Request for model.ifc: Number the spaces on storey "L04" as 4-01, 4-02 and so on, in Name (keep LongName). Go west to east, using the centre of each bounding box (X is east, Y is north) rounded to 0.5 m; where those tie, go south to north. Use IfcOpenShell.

First a look at what the model holds.

```python
import ifcopenshell
import ifcopenshell.util.element
import ifcopenshell.util.placement

model = ifcopenshell.open("model.ifc")
print(model.schema)
storey = next(s for s in model.by_type("IfcBuildingStorey") if s.Name == "L04")
spaces = [e for e in ifcopenshell.util.element.get_decomposition(storey) if e.is_a("IfcSpace")]
for e in sorted(spaces, key=lambda e: e.id()):
    origin = ifcopenshell.util.placement.get_local_placement(e.ObjectPlacement)[:3, 3]
    print(e.id(), e.Name, e.LongName, origin.round(2) + 0.0, sep=" | ")
```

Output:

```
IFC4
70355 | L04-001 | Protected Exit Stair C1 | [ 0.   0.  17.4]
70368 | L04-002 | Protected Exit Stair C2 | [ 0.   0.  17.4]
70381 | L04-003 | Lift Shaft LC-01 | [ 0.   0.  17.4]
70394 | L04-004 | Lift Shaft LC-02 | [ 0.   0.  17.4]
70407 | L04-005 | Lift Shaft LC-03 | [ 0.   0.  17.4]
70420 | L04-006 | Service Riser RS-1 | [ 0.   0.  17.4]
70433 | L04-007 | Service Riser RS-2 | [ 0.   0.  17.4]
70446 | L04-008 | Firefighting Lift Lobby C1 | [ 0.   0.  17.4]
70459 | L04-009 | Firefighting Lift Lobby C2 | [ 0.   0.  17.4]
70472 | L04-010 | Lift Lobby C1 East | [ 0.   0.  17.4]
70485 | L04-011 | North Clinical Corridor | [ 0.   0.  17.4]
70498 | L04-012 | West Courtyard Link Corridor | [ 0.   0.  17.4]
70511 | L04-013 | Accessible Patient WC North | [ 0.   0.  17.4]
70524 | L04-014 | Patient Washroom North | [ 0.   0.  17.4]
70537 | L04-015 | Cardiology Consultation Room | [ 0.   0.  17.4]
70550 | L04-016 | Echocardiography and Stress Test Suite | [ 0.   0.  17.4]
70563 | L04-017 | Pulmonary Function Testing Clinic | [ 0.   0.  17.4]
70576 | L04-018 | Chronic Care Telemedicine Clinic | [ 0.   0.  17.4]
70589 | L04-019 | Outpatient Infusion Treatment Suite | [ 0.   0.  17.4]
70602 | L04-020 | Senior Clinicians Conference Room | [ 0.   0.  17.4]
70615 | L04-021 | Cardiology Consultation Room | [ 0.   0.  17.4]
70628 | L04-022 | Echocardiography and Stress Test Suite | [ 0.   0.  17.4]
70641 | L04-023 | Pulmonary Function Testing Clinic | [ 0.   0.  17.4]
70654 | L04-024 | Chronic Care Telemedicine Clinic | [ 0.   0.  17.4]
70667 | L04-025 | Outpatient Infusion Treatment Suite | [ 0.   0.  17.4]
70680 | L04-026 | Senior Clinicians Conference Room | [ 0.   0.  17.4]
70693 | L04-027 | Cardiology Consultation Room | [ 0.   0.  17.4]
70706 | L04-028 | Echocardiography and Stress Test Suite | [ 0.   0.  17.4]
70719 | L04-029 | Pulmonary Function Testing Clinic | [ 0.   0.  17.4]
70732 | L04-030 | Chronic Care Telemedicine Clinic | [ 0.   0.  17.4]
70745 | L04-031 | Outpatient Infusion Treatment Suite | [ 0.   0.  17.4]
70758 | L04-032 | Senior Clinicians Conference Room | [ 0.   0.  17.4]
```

```python
import ifcopenshell
import ifcopenshell.geom
import ifcopenshell.util.element
import ifcopenshell.util.shape

model = ifcopenshell.open("model.ifc")
settings = ifcopenshell.geom.settings()
settings.set("use-world-coords", True)


def centre(element):
    shape = ifcopenshell.geom.create_shape(settings, element)
    return ifcopenshell.util.shape.get_bbox_centroid(shape.geometry)


storey = next(s for s in model.by_type("IfcBuildingStorey") if s.Name == "L04")
spaces = [e for e in ifcopenshell.util.element.get_decomposition(storey) if e.is_a("IfcSpace")]

# Insertion points can sit at a corner or the storey origin, so sort by the geometry (in metres).
centres = {e: centre(e) for e in spaces}
spaces.sort(key=lambda e: (round(centres[e][0] / 0.5), centres[e][1]))

for i, e in enumerate(spaces, start=1):
    number = f"4-{i:02d}"
    e.Name = number
    print(e.id(), number)

model.write("model_updated.ifc")
```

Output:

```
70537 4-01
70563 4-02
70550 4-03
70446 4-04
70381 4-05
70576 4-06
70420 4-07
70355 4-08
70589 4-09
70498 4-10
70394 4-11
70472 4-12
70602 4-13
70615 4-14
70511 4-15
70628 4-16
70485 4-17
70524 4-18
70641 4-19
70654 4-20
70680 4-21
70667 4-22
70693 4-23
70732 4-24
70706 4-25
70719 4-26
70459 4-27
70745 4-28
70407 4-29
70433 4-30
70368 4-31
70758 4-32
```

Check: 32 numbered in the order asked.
